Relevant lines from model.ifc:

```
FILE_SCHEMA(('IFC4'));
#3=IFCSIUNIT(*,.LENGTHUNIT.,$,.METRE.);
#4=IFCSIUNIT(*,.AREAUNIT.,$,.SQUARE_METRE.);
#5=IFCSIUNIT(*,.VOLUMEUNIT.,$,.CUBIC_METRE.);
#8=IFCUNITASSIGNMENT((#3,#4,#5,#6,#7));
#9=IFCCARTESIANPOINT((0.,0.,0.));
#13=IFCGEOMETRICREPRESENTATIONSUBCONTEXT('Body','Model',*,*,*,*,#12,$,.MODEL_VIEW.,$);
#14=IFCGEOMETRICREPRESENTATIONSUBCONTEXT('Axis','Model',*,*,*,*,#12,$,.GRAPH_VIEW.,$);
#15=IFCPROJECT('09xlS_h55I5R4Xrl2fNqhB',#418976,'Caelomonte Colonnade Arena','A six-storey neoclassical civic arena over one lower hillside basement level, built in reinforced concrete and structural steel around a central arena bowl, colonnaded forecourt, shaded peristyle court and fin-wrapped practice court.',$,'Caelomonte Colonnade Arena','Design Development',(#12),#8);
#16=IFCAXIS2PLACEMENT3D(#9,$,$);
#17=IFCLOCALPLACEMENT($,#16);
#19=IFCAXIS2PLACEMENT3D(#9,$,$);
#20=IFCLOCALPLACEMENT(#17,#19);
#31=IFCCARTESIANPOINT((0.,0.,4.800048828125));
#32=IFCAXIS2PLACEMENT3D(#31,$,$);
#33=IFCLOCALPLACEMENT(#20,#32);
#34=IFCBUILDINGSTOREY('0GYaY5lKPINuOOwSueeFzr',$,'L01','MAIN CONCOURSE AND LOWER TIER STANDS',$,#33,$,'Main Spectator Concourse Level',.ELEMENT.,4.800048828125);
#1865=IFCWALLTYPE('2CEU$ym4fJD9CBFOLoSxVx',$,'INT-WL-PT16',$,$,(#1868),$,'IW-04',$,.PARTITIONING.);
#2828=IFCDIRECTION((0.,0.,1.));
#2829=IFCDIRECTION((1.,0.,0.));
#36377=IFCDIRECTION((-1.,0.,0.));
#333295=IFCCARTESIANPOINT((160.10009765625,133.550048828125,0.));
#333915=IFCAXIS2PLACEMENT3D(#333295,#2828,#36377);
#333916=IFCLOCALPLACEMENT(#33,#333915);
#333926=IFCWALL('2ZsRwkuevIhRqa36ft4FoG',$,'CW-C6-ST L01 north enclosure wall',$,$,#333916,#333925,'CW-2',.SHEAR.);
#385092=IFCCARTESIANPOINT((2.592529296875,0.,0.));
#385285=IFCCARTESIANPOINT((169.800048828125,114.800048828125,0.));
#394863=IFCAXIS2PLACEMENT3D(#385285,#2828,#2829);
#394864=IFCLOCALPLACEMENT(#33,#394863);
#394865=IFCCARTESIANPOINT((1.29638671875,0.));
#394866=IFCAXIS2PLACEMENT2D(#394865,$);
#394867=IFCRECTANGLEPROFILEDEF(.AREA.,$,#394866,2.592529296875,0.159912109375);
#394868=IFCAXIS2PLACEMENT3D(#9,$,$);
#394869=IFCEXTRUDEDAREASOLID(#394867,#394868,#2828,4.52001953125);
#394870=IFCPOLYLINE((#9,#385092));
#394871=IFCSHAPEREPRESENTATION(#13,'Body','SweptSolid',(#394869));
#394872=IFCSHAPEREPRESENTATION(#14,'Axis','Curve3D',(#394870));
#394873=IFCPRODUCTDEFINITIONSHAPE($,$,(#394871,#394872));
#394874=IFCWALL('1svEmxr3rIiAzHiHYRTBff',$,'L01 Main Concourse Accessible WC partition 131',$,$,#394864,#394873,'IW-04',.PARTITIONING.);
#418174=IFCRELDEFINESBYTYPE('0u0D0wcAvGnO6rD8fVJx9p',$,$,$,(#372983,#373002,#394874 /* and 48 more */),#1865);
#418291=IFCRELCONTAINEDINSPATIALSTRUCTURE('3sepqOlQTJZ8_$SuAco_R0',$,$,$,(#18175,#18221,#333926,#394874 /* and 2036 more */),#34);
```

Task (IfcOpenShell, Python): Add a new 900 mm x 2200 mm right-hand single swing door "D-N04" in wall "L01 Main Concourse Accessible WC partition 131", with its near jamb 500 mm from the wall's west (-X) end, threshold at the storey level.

```python
import numpy as np
import ifcopenshell
import ifcopenshell.api.feature
import ifcopenshell.api.geometry
import ifcopenshell.api.root
import ifcopenshell.api.spatial
import ifcopenshell.geom
import ifcopenshell.util.element
import ifcopenshell.util.placement
import ifcopenshell.util.representation
import ifcopenshell.util.shape
import ifcopenshell.util.unit

model = ifcopenshell.open("model.ifc")
unit_scale = ifcopenshell.util.unit.calculate_unit_scale(model)
settings = ifcopenshell.geom.settings()


def volume(element):
    """Net volume in cubic metres, openings subtracted."""
    shape = ifcopenshell.geom.create_shape(settings, element)
    return ifcopenshell.util.shape.get_volume(shape.geometry)


wall = model.by_guid("1svEmxr3rIiAzHiHYRTBff")
storey = ifcopenshell.util.element.get_container(wall, ifc_class="IfcBuildingStorey")
context = ifcopenshell.util.representation.get_context(model, "Model", "Body", "MODEL_VIEW")
before = volume(wall)

width, height, from_end, sill = 0.9, 2.2, 0.5, 0.0  # metres

# The wall runs along its own X axis, and the end named is its -X end.
wall_shape = ifcopenshell.geom.create_shape(settings, wall)
x, y, z = ifcopenshell.util.shape.get_vertices(wall_shape.geometry).T
start = x.min() + from_end
face, thickness = float(y.min()), float(y.max() - y.min())
wall_matrix = ifcopenshell.util.placement.get_local_placement(wall.ObjectPlacement)
level = ifcopenshell.util.placement.get_local_placement(storey.ObjectPlacement)[2, 3]


def in_wall(x, y):
    """Placement at x, y metres in the wall's axes, at sill height."""
    matrix = wall_matrix.copy()
    matrix[:, 3] = wall_matrix @ np.array([x / unit_scale, y / unit_scale, 0.0, 1.0])
    matrix[2, 3] = level + sill / unit_scale
    return matrix


# Opening: a box that overshoots both wall faces by 50 mm.
opening = ifcopenshell.api.root.create_entity(model, ifc_class="IfcOpeningElement", predefined_type="OPENING")
box = ifcopenshell.api.geometry.add_wall_representation(
    model, context=context, length=width, height=height, thickness=thickness + 0.1
)
ifcopenshell.api.geometry.assign_representation(model, product=opening, representation=box)
ifcopenshell.api.geometry.edit_object_placement(model, product=opening, matrix=in_wall(start, face - 0.05), is_si=False)
ifcopenshell.api.feature.add_feature(model, feature=opening, element=wall)

door = ifcopenshell.api.root.create_entity(model, ifc_class="IfcDoor", name="D-N04", predefined_type="DOOR")
door.OverallWidth, door.OverallHeight = width / unit_scale, height / unit_scale
door.OperationType = "SINGLE_SWING_RIGHT"
body = ifcopenshell.api.geometry.add_door_representation(
    model,
    context=context,
    overall_width=door.OverallWidth,
    overall_height=door.OverallHeight,
    operation_type="SINGLE_SWING_RIGHT",
    lining_properties={"LiningDepth": thickness / unit_scale, "ThresholdDepth": thickness / unit_scale},
)
ifcopenshell.api.geometry.assign_representation(model, product=door, representation=body)
ifcopenshell.api.spatial.assign_container(model, products=[door], relating_structure=storey)
ifcopenshell.api.feature.add_filling(model, opening=opening, element=door)

# The lining spans the wall, so the door starts at the wall face.
ifcopenshell.api.geometry.edit_object_placement(model, product=door, matrix=in_wall(start, face), is_si=False)

after = volume(wall)

print(f"wall volume {before:.3f} -> {after:.3f} m3")

model.write("model_rev.ifc")
```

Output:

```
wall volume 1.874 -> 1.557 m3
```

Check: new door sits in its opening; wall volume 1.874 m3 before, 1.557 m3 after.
